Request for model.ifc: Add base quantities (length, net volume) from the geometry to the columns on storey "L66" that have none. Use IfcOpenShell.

First a look at what the model holds.

```python
import ifcopenshell
import ifcopenshell.util.element
import ifcopenshell.util.unit

model = ifcopenshell.open("model.ifc")
print(model.schema)
for unit_type in ("LENGTHUNIT", "AREAUNIT", "VOLUMEUNIT"):
    print(unit_type, ifcopenshell.util.unit.calculate_unit_scale(model, unit_type))
storey = next(s for s in model.by_type("IfcBuildingStorey") if s.Name == "L66")
columns = [e for e in ifcopenshell.util.element.get_decomposition(storey) if e.is_a("IfcColumn")]
for e in sorted(columns, key=lambda e: e.id()):
    print(e.id(), e.is_a(), e.Name, list(ifcopenshell.util.element.get_psets(e, qtos_only=True)), sep=" | ")
```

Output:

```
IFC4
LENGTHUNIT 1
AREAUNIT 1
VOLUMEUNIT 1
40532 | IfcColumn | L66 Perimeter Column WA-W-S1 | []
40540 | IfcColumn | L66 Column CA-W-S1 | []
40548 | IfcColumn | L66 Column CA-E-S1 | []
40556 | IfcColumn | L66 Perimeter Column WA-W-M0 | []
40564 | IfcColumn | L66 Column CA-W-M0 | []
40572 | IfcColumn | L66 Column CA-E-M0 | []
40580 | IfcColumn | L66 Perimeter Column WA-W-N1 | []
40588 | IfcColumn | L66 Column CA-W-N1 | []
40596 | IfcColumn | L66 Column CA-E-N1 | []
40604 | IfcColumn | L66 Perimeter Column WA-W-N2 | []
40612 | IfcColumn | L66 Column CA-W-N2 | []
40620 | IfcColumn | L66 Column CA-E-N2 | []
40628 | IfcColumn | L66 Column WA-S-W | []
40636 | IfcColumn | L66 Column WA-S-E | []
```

```python
import ifcopenshell
import ifcopenshell.api.pset
import ifcopenshell.geom
import ifcopenshell.util.element
import ifcopenshell.util.shape
import ifcopenshell.util.unit

model = ifcopenshell.open("model.ifc")
unit_scale = ifcopenshell.util.unit.calculate_unit_scale(model)
volume_scale = ifcopenshell.util.unit.calculate_unit_scale(model, "VOLUMEUNIT")
settings = ifcopenshell.geom.settings()

storey = next(s for s in model.by_type("IfcBuildingStorey") if s.Name == "L66")
columns = [e for e in ifcopenshell.util.element.get_decomposition(storey) if e.is_a("IfcColumn")]

for e in sorted(columns, key=lambda e: e.id()):
    if ifcopenshell.util.element.get_psets(e, qtos_only=True, should_inherit=False):
        continue
    # Geometry comes back in metres, in the element's own axes.
    shape = ifcopenshell.geom.create_shape(settings, e)
    values = {
        "Length": ifcopenshell.util.shape.get_z(shape.geometry) / unit_scale,
        "NetVolume": ifcopenshell.util.shape.get_volume(shape.geometry) / volume_scale,
    }
    qto = ifcopenshell.api.pset.add_qto(model, product=e, name="Qto_ColumnBaseQuantities")
    ifcopenshell.api.pset.edit_qto(model, qto=qto, properties=values)
    print(e.id(), {k: round(v, 3) for k, v in values.items()})

model.write("model_rev.ifc")
```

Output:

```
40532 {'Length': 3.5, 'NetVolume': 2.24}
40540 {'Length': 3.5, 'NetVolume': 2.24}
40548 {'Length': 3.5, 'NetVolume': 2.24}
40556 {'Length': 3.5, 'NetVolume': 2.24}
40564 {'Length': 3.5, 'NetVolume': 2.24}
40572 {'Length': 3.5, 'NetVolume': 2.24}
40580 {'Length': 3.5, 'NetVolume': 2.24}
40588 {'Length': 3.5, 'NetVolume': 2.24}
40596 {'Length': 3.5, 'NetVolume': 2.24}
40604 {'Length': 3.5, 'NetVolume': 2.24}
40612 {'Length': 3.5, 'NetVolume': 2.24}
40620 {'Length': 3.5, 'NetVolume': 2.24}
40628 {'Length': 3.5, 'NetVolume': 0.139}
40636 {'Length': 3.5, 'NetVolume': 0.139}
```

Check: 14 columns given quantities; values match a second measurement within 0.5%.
